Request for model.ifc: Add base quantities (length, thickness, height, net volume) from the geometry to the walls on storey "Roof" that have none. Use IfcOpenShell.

First a look at what the model holds.

```python
import ifcopenshell
import ifcopenshell.util.element
import ifcopenshell.util.unit

model = ifcopenshell.open("model.ifc")
print(model.schema)
for unit_type in ("LENGTHUNIT", "AREAUNIT", "VOLUMEUNIT"):
    print(unit_type, ifcopenshell.util.unit.calculate_unit_scale(model, unit_type))
storey = next(s for s in model.by_type("IfcBuildingStorey") if s.Name == "Roof")
walls = [e for e in ifcopenshell.util.element.get_decomposition(storey) if e.is_a("IfcWall")]
for e in sorted(walls, key=lambda e: e.id()):
    print(e.id(), e.is_a(), e.Name, list(ifcopenshell.util.element.get_psets(e, qtos_only=True)), sep=" | ")
```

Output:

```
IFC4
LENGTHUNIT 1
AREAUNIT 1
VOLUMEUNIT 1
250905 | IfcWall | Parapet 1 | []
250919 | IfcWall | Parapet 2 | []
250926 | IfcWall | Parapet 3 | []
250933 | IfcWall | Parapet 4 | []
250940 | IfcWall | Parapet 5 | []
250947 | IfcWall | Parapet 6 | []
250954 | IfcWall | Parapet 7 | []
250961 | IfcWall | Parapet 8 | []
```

```python
import ifcopenshell
import ifcopenshell.api.pset
import ifcopenshell.geom
import ifcopenshell.util.element
import ifcopenshell.util.shape
import ifcopenshell.util.unit

model = ifcopenshell.open("model.ifc")
unit_scale = ifcopenshell.util.unit.calculate_unit_scale(model)
volume_scale = ifcopenshell.util.unit.calculate_unit_scale(model, "VOLUMEUNIT")
settings = ifcopenshell.geom.settings()

storey = next(s for s in model.by_type("IfcBuildingStorey") if s.Name == "Roof")
walls = [e for e in ifcopenshell.util.element.get_decomposition(storey) if e.is_a("IfcWall")]

for e in sorted(walls, key=lambda e: e.id()):
    if ifcopenshell.util.element.get_psets(e, qtos_only=True, should_inherit=False):
        continue
    # Geometry comes back in metres, in the element's own axes.
    shape = ifcopenshell.geom.create_shape(settings, e)
    values = {
        "Length": ifcopenshell.util.shape.get_x(shape.geometry) / unit_scale,
        "Width": ifcopenshell.util.shape.get_y(shape.geometry) / unit_scale,
        "Height": ifcopenshell.util.shape.get_z(shape.geometry) / unit_scale,
        "NetVolume": ifcopenshell.util.shape.get_volume(shape.geometry) / volume_scale,
    }
    qto = ifcopenshell.api.pset.add_qto(model, product=e, name="Qto_WallBaseQuantities")
    ifcopenshell.api.pset.edit_qto(model, qto=qto, properties=values)
    print(e.id(), {k: round(v, 3) for k, v in values.items()})

model.write("model_v2.ifc")
```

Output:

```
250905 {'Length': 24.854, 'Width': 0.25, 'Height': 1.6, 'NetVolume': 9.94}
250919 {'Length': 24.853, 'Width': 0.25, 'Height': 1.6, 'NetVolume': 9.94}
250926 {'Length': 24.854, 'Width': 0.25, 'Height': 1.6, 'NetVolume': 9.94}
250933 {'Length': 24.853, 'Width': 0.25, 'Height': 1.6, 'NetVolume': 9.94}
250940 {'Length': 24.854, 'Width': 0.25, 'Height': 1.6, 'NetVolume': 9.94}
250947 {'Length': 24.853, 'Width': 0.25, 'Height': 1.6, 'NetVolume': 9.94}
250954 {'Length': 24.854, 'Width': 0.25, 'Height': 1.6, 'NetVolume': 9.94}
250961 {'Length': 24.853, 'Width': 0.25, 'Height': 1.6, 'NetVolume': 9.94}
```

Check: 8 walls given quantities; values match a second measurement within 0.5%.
